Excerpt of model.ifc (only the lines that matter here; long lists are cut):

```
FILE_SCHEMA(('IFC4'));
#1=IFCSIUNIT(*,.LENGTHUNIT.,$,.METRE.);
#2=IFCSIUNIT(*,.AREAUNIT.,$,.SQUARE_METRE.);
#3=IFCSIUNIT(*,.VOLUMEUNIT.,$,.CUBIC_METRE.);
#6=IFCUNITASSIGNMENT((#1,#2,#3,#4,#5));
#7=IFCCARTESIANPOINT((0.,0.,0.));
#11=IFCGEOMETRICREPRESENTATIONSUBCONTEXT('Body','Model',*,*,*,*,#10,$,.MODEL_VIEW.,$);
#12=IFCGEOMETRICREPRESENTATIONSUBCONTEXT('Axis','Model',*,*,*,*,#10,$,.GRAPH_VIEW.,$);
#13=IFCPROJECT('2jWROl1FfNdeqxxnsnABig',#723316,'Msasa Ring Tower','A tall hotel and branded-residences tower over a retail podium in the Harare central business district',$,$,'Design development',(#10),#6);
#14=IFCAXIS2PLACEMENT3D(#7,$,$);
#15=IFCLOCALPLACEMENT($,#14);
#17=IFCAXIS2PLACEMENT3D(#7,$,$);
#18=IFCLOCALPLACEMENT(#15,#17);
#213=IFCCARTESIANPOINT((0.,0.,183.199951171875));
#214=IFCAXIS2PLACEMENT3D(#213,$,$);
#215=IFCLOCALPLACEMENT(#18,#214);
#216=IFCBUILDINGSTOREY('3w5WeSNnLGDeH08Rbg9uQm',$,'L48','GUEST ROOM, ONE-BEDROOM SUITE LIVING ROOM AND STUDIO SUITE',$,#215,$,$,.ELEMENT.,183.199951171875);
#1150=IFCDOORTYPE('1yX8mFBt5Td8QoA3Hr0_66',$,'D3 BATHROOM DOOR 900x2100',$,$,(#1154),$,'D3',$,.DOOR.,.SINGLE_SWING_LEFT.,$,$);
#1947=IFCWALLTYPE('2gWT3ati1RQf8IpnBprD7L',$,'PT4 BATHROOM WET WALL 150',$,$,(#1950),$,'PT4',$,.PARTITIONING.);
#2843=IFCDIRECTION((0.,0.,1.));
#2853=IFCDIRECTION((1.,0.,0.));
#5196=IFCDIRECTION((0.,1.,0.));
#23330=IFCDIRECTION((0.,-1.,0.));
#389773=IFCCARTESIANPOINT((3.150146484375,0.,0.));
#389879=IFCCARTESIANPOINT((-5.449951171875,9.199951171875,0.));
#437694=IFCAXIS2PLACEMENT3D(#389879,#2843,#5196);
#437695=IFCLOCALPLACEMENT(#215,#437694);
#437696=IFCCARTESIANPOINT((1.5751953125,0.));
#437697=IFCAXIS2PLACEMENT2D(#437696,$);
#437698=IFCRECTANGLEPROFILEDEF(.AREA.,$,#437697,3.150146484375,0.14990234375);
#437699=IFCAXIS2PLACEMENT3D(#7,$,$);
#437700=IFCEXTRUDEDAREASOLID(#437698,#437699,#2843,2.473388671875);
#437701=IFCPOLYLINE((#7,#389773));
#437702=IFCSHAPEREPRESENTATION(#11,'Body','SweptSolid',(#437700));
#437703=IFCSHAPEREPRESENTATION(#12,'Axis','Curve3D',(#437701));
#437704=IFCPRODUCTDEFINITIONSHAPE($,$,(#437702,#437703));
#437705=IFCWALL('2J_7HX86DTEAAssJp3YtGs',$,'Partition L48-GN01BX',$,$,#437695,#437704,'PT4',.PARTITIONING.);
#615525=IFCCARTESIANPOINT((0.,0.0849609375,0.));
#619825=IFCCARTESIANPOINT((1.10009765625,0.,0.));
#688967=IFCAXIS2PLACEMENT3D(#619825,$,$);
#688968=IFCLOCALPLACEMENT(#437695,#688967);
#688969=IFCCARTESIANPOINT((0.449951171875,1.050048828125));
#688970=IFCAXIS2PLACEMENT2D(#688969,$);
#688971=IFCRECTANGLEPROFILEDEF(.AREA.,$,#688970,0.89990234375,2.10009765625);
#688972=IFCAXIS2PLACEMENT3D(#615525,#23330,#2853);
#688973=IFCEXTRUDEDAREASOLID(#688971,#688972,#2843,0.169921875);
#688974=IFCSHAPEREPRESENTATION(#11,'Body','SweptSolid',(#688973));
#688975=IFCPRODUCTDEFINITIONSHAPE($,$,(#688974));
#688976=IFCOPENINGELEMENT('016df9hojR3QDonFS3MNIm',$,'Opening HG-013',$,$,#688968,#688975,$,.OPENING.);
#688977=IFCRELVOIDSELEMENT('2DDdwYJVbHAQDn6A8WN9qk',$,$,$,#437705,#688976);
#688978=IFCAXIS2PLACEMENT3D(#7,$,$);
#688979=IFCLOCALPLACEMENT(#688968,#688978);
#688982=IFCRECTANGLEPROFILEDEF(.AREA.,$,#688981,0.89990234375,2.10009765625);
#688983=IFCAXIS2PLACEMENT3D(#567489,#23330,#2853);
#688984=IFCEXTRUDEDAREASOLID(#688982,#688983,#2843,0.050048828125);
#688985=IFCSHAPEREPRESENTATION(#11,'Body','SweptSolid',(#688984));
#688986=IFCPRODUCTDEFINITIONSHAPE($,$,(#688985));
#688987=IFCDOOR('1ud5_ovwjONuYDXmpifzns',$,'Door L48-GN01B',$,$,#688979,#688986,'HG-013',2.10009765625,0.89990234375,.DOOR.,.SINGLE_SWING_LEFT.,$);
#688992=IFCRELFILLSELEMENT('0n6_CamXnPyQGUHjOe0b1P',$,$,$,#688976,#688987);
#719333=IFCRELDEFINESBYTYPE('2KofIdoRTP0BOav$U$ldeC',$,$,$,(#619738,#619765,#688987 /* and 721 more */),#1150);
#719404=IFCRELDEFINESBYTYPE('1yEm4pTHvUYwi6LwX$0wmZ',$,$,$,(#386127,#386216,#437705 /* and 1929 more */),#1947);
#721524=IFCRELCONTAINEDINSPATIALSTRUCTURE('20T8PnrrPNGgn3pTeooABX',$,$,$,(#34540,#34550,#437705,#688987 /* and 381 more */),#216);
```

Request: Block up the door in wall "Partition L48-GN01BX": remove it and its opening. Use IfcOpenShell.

```python
import ifcopenshell
import ifcopenshell.api.feature
import ifcopenshell.api.root
import ifcopenshell.geom
import ifcopenshell.util.shape

model = ifcopenshell.open("model.ifc")
settings = ifcopenshell.geom.settings()


def volume(element):
    """Net volume in cubic metres, openings subtracted."""
    shape = ifcopenshell.geom.create_shape(settings, element)
    return ifcopenshell.util.shape.get_volume(shape.geometry)


door = model.by_guid("1ud5_ovwjONuYDXmpifzns")
opening = door.FillsVoids[0].RelatingOpeningElement
wall = opening.VoidsElements[0].RelatingBuildingElement
before = volume(wall)

ifcopenshell.api.root.remove_product(model, product=door)
ifcopenshell.api.feature.remove_feature(model, feature=opening)

after = volume(wall)

print(f"wall volume {before:.3f} -> {after:.3f} m3")

model.write("model_v2.ifc")
```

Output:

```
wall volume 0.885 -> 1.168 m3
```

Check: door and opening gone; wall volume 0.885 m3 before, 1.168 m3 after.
